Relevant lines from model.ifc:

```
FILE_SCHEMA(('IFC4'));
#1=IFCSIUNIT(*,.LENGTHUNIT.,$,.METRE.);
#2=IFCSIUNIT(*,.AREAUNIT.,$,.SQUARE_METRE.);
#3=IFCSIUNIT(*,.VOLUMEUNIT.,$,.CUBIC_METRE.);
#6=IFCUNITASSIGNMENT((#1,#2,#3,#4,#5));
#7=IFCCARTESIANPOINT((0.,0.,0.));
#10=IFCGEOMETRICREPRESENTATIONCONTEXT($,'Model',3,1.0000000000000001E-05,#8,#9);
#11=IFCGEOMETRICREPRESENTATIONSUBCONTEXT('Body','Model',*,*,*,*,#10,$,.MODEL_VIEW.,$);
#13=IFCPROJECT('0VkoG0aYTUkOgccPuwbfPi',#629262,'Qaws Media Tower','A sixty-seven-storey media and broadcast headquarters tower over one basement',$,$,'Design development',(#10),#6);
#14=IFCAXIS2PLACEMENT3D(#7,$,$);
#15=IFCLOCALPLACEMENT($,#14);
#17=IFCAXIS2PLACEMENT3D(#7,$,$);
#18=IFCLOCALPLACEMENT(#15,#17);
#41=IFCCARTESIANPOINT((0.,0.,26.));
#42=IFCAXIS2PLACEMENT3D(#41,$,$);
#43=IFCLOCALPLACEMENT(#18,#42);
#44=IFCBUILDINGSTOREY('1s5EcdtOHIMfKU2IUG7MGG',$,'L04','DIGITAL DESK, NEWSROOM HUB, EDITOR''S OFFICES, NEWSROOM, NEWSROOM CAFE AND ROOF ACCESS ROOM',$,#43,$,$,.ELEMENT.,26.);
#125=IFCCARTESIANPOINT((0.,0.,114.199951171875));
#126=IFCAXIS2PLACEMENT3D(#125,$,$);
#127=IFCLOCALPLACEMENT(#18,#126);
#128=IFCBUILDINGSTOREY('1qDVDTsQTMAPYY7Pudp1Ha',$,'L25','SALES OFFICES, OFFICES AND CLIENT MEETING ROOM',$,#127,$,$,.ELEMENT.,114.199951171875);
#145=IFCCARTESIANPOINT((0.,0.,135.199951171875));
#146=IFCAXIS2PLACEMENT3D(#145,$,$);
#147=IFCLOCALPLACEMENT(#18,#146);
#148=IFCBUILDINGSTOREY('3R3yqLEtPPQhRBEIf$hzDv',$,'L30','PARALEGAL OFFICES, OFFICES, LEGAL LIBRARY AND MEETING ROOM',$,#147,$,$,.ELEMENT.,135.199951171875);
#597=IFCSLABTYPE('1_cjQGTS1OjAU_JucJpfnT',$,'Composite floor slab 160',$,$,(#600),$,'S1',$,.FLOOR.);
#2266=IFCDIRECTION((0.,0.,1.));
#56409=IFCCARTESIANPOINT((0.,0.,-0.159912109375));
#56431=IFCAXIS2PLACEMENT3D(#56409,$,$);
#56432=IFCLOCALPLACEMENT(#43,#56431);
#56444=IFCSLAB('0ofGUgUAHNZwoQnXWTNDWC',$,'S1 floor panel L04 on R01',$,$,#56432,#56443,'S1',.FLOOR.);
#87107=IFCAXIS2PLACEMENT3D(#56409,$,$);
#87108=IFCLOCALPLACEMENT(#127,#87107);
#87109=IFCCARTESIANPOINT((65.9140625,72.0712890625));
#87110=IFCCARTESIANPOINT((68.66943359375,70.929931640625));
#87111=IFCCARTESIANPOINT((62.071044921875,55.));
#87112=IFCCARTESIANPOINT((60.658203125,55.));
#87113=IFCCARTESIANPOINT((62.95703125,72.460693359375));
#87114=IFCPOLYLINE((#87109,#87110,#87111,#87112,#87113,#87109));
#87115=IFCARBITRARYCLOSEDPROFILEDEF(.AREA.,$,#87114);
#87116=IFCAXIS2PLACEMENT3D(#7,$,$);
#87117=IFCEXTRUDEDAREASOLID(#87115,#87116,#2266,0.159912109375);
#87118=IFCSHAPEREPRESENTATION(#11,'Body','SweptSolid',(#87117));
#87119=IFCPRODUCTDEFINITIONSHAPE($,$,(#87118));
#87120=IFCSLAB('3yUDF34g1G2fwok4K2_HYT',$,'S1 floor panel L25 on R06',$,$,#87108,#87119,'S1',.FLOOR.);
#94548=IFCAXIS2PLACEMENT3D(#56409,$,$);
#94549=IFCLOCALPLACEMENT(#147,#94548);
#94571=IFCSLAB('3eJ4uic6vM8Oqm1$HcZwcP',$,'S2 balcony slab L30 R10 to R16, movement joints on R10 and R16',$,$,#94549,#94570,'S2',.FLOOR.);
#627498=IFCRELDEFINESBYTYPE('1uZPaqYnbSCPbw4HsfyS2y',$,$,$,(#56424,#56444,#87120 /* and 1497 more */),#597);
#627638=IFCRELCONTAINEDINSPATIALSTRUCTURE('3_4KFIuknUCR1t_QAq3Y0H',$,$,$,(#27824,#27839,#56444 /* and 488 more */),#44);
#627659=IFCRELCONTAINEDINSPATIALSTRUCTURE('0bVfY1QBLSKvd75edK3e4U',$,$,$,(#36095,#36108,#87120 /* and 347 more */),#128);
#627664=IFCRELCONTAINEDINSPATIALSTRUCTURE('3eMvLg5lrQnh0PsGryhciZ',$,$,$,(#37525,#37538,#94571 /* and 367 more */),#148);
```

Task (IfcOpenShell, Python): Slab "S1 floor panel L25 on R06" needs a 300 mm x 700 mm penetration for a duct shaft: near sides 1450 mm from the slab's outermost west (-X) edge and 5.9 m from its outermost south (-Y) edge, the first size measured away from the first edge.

```python
import numpy as np
import ifcopenshell
import ifcopenshell.api.feature
import ifcopenshell.api.geometry
import ifcopenshell.api.root
import ifcopenshell.geom
import ifcopenshell.util.placement
import ifcopenshell.util.representation
import ifcopenshell.util.shape
import ifcopenshell.util.unit

model = ifcopenshell.open("model.ifc")
unit_scale = ifcopenshell.util.unit.calculate_unit_scale(model)
settings = ifcopenshell.geom.settings()


def volume(element):
    """Net volume in cubic metres, openings subtracted."""
    shape = ifcopenshell.geom.create_shape(settings, element)
    return ifcopenshell.util.shape.get_volume(shape.geometry)


slab = model.by_id(87120)
before = volume(slab)

# Extent in the slab's own axes, in metres. The edges named are its -X and -Y sides.
slab_shape = ifcopenshell.geom.create_shape(settings, slab)
vertices = ifcopenshell.util.shape.get_vertices(slab_shape.geometry)
x_min, y_min, bottom = vertices.min(axis=0)
top = vertices[:, 2].max()

opening = ifcopenshell.api.root.create_entity(model, ifc_class="IfcOpeningElement", name="Duct shaft opening", predefined_type="OPENING")
context = ifcopenshell.util.representation.get_context(model, "Model", "Body", "MODEL_VIEW")
width, depth = 0.3, 0.7
outline = [(0.0, 0.0), (width, 0.0), (width, depth), (0.0, depth), (0.0, 0.0)]
# Overshoot both faces by 50 mm so the cut is clean.
shape = ifcopenshell.api.geometry.add_slab_representation(
    model, context=context, depth=top - bottom + 0.1, polyline=outline
)
ifcopenshell.api.geometry.assign_representation(model, product=opening, representation=shape)

matrix = ifcopenshell.util.placement.get_local_placement(slab.ObjectPlacement)
matrix[:, 3] = matrix @ np.append(np.array([x_min + 1.45, y_min + 5.9, bottom - 0.05]) / unit_scale, 1.0)
ifcopenshell.api.geometry.edit_object_placement(model, product=opening, matrix=matrix, is_si=False)
ifcopenshell.api.feature.add_feature(model, feature=opening, element=slab)

after = volume(slab)

print(f"slab volume {before:.3f} -> {after:.3f} m3")

model.write("model_updated.ifc")
```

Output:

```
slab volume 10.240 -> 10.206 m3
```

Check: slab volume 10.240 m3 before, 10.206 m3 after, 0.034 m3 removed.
